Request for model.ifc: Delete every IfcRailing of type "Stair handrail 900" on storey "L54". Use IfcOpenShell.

First a look at what the model holds.

```python
import ifcopenshell
import ifcopenshell.util.element

model = ifcopenshell.open("model.ifc")
print(model.schema)
storey = next(s for s in model.by_type("IfcBuildingStorey") if s.Name == "L54")
railings = [e for e in ifcopenshell.util.element.get_decomposition(storey) if e.is_a("IfcRailing")]
seen = {}
for e in railings:
    element_type = ifcopenshell.util.element.get_type(e)
    name = element_type.Name if element_type not in (None, e) else None
    seen[name] = seen.get(name, 0) + 1
for name, count in sorted(seen.items(), key=str):
    print(count, "x", name)
```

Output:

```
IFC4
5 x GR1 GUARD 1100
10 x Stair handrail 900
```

```python
import ifcopenshell
import ifcopenshell.api.root
import ifcopenshell.util.element

model = ifcopenshell.open("model.ifc")

storey = next(s for s in model.by_type("IfcBuildingStorey") if s.Name == "L54")
railings = [e for e in ifcopenshell.util.element.get_decomposition(storey) if e.is_a("IfcRailing")]
targets = [e for e in railings if (t := ifcopenshell.util.element.get_type(e)) not in (None, e) and t.Name == "Stair handrail 900"]

for e in targets:
    ifcopenshell.api.root.remove_product(model, product=e)
print(len(targets), "removed")

model.write("model-out.ifc")
```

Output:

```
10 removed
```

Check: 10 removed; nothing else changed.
